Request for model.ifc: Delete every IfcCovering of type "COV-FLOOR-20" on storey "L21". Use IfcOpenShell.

First a look at what the model holds.

```python
import ifcopenshell
import ifcopenshell.util.element

model = ifcopenshell.open("model.ifc")
print(model.schema)
storey = next(s for s in model.by_type("IfcBuildingStorey") if s.Name == "L21")
coverings = [e for e in ifcopenshell.util.element.get_decomposition(storey) if e.is_a("IfcCovering")]
seen = {}
for e in coverings:
    element_type = ifcopenshell.util.element.get_type(e)
    name = element_type.Name if element_type not in (None, e) else None
    seen[name] = seen.get(name, 0) + 1
for name, count in sorted(seen.items(), key=str):
    print(count, "x", name)
```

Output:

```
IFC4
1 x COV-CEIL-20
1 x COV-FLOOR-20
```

```python
import ifcopenshell
import ifcopenshell.api.root
import ifcopenshell.util.element

model = ifcopenshell.open("model.ifc")

storey = next(s for s in model.by_type("IfcBuildingStorey") if s.Name == "L21")
coverings = [e for e in ifcopenshell.util.element.get_decomposition(storey) if e.is_a("IfcCovering")]
targets = [e for e in coverings if (t := ifcopenshell.util.element.get_type(e)) not in (None, e) and t.Name == "COV-FLOOR-20"]

for e in targets:
    ifcopenshell.api.root.remove_product(model, product=e)
print(len(targets), "removed")

model.write("model_edited.ifc")
```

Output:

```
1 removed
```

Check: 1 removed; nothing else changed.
